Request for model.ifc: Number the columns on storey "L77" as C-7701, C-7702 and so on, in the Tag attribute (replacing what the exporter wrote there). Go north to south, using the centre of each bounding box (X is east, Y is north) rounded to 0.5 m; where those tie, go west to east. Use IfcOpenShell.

First a look at what the model holds.

```python
import ifcopenshell
import ifcopenshell.util.element
import ifcopenshell.util.placement

model = ifcopenshell.open("model.ifc")
print(model.schema)
storey = next(s for s in model.by_type("IfcBuildingStorey") if s.Name == "L77")
columns = [e for e in ifcopenshell.util.element.get_decomposition(storey) if e.is_a("IfcColumn")]
for e in sorted(columns, key=lambda e: e.id()):
    origin = ifcopenshell.util.placement.get_local_placement(e.ObjectPlacement)[:3, 3]
    print(e.id(), e.Tag, e.Name, origin.round(2) + 0.0, sep=" | ")
```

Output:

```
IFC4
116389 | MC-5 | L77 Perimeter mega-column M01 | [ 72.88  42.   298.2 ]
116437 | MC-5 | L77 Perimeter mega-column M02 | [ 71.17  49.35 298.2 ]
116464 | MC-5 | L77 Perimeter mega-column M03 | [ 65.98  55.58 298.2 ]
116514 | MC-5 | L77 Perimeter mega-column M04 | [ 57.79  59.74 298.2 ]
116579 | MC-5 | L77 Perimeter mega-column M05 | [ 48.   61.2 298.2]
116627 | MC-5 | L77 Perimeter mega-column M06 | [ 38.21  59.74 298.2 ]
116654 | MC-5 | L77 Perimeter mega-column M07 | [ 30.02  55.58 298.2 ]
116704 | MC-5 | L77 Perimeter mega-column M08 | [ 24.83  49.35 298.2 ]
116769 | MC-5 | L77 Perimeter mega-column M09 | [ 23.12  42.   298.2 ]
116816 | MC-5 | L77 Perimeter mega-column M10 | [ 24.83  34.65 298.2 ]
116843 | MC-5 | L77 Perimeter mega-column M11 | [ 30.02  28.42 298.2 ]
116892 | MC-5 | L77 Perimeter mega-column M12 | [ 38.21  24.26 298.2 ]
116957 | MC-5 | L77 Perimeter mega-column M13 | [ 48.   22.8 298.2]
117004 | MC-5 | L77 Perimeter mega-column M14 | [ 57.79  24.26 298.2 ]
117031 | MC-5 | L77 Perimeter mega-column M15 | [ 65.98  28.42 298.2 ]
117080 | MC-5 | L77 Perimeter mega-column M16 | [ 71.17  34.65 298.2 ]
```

```python
import ifcopenshell
import ifcopenshell.geom
import ifcopenshell.util.element
import ifcopenshell.util.shape

model = ifcopenshell.open("model.ifc")
settings = ifcopenshell.geom.settings()
settings.set("use-world-coords", True)


def centre(element):
    shape = ifcopenshell.geom.create_shape(settings, element)
    return ifcopenshell.util.shape.get_bbox_centroid(shape.geometry)


storey = next(s for s in model.by_type("IfcBuildingStorey") if s.Name == "L77")
columns = [e for e in ifcopenshell.util.element.get_decomposition(storey) if e.is_a("IfcColumn")]

# Insertion points can sit at a corner or the storey origin, so sort by the geometry (in metres).
centres = {e: centre(e) for e in columns}
columns.sort(key=lambda e: (-round(centres[e][1] / 0.5), centres[e][0]))

for i, e in enumerate(columns, start=1):
    number = f"C-77{i:02d}"
    e.Tag = number
    print(e.id(), number)

model.write("model_rev.ifc")
```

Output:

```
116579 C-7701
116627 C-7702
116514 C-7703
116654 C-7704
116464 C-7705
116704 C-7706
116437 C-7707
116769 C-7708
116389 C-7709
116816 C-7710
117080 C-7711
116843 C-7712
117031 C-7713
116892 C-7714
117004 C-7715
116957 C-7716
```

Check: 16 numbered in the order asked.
